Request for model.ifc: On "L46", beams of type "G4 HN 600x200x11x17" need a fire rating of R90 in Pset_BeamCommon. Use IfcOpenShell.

First a look at what the model holds.

```python
import ifcopenshell
import ifcopenshell.util.element

model = ifcopenshell.open("model.ifc")
print(model.schema)
storey = next(s for s in model.by_type("IfcBuildingStorey") if s.Name == "L46")
beams = [e for e in ifcopenshell.util.element.get_decomposition(storey) if e.is_a("IfcBeam")]
seen = {}
for e in beams:
    element_type = ifcopenshell.util.element.get_type(e)
    key = (element_type.Name if element_type != e and element_type else None, ifcopenshell.util.element.get_pset(e, "Pset_BeamCommon", "FireRating"))
    seen[key] = seen.get(key, 0) + 1
for (name, value), count in sorted(seen.items(), key=str):
    print(count, "x", name, "|", value)
```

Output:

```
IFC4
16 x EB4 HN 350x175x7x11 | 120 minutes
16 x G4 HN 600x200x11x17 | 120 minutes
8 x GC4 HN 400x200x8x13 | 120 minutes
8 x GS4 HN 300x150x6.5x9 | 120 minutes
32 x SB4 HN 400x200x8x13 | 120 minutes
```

```python
import ifcopenshell
import ifcopenshell.api.pset
import ifcopenshell.util.element

model = ifcopenshell.open("model.ifc")

storey = next(s for s in model.by_type("IfcBuildingStorey") if s.Name == "L46")
beams = [e for e in ifcopenshell.util.element.get_decomposition(storey) if e.is_a("IfcBeam")]

count = 0
for e in beams:
    element_type = ifcopenshell.util.element.get_type(e)
    if element_type in (None, e) or element_type.Name != "G4 HN 600x200x11x17":
        continue
    found = ifcopenshell.util.element.get_pset(e, "Pset_BeamCommon", should_inherit=False)
    if found:
        pset = model.by_id(found["id"])
        if len(ifcopenshell.util.element.get_elements_by_pset(pset)) > 1:
            pset = ifcopenshell.api.pset.unshare_pset(model, products=[e], pset=pset)[0]
    else:
        pset = ifcopenshell.api.pset.add_pset(model, product=e, name="Pset_BeamCommon")
    ifcopenshell.api.pset.edit_pset(model, pset=pset, properties={"FireRating": "R90"})
    count += 1

print(count, "beams updated")

model.write("model_rev.ifc")
```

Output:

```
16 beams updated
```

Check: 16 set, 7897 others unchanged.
